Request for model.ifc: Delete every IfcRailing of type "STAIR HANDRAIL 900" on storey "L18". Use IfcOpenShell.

First a look at what the model holds.

```python
import ifcopenshell
import ifcopenshell.util.element

model = ifcopenshell.open("model.ifc")
print(model.schema)
storey = next(s for s in model.by_type("IfcBuildingStorey") if s.Name == "L18")
railings = [e for e in ifcopenshell.util.element.get_decomposition(storey) if e.is_a("IfcRailing")]
seen = {}
for e in railings:
    element_type = ifcopenshell.util.element.get_type(e)
    name = element_type.Name if element_type not in (None, e) else None
    seen[name] = seen.get(name, 0) + 1
for name, count in sorted(seen.items(), key=str):
    print(count, "x", name)
```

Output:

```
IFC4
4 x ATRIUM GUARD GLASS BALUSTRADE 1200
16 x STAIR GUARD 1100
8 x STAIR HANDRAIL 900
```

```python
import ifcopenshell
import ifcopenshell.api.root
import ifcopenshell.util.element

model = ifcopenshell.open("model.ifc")

storey = next(s for s in model.by_type("IfcBuildingStorey") if s.Name == "L18")
railings = [e for e in ifcopenshell.util.element.get_decomposition(storey) if e.is_a("IfcRailing")]
targets = [e for e in railings if (t := ifcopenshell.util.element.get_type(e)) not in (None, e) and t.Name == "STAIR HANDRAIL 900"]

for e in targets:
    ifcopenshell.api.root.remove_product(model, product=e)
print(len(targets), "removed")

model.write("model_rev.ifc")
```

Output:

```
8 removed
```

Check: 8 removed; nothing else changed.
